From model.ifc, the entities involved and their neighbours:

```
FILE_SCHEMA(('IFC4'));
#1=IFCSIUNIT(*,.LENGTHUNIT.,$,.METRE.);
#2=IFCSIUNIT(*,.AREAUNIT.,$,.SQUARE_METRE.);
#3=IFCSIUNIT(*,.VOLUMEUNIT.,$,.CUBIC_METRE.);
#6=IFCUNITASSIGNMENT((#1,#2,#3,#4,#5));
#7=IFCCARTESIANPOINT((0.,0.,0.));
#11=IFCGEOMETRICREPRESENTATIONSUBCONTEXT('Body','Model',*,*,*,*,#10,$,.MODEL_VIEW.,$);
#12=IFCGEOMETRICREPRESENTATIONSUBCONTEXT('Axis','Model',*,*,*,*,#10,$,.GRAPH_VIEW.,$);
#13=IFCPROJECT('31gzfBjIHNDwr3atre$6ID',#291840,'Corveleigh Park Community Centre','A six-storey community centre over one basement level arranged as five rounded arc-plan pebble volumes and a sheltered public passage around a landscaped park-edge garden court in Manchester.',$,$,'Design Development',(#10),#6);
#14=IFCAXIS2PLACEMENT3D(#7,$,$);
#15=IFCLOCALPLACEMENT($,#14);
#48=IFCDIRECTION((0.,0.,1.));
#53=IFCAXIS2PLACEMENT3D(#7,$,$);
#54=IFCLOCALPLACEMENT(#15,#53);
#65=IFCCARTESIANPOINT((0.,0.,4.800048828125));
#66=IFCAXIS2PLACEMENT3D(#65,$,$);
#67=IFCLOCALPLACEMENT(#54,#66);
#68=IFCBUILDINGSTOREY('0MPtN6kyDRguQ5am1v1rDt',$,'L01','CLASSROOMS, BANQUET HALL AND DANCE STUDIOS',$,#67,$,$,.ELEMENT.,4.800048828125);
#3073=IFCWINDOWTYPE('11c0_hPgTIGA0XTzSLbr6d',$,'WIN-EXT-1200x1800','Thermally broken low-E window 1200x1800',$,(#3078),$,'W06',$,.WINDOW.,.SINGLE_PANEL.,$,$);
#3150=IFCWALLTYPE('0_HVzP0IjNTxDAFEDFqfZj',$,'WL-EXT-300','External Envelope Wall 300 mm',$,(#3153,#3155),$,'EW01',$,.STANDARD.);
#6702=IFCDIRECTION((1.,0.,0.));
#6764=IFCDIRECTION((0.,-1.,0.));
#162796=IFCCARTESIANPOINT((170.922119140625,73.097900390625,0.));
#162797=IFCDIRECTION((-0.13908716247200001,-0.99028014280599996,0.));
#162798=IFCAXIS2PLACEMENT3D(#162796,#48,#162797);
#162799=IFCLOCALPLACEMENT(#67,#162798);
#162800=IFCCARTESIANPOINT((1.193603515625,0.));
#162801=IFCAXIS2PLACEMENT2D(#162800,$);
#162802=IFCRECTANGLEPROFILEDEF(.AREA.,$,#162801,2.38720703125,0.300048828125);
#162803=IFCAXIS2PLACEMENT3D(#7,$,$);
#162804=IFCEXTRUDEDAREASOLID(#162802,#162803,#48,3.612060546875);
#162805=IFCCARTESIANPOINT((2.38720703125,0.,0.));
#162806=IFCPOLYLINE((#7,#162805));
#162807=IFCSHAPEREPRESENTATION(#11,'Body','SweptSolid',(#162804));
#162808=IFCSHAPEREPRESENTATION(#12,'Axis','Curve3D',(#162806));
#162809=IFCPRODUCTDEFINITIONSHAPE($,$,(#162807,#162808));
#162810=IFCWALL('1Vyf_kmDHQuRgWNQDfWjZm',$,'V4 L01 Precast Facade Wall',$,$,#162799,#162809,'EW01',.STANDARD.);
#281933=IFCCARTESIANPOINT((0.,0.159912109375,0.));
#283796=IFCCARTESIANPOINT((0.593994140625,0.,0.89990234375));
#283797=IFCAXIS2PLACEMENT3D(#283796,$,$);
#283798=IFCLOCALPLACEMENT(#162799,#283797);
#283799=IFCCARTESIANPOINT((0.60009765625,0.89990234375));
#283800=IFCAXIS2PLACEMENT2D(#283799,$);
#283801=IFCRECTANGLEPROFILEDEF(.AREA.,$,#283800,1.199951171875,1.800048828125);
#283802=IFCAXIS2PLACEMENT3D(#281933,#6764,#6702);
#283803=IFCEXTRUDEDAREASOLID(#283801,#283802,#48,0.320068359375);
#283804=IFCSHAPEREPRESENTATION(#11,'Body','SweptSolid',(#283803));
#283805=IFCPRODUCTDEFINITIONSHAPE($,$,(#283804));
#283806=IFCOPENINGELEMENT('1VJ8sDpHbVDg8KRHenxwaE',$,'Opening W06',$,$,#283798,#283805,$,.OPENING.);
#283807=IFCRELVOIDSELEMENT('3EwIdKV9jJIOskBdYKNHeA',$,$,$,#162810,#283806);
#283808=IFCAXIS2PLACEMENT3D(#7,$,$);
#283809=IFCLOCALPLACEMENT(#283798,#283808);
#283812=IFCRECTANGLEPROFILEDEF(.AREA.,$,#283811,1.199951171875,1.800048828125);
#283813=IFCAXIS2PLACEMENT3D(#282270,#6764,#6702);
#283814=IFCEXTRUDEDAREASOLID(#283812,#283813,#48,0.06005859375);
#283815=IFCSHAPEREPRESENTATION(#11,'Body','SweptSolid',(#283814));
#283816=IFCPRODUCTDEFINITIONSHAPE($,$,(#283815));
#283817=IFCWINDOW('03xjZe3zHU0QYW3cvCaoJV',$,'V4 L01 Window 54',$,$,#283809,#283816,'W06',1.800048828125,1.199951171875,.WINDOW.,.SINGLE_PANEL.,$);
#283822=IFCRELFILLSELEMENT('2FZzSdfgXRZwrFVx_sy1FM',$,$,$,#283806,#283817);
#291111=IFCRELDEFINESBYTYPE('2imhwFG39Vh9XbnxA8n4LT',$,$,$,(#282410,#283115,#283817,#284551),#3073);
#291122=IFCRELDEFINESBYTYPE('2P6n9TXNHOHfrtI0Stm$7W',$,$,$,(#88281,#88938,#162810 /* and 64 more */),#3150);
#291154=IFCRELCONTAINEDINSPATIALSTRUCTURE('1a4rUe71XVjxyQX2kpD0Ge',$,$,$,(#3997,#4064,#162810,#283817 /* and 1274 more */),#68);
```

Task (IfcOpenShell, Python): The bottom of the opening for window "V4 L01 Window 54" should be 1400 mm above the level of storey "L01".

```python
import numpy as np
import ifcopenshell
import ifcopenshell.api.geometry
import ifcopenshell.geom
import ifcopenshell.util.element
import ifcopenshell.util.placement
import ifcopenshell.util.shape
import ifcopenshell.util.unit

model = ifcopenshell.open("model.ifc")
unit_scale = ifcopenshell.util.unit.calculate_unit_scale(model)

window = model.by_guid("03xjZe3zHU0QYW3cvCaoJV")
opening = window.FillsVoids[0].RelatingOpeningElement
storey = ifcopenshell.util.element.get_container(window, ifc_class="IfcBuildingStorey")
level = ifcopenshell.util.placement.get_local_placement(storey.ObjectPlacement)[2, 3]

# The opening's origin need not be at the sill, so measure its lowest point.
shape = ifcopenshell.geom.create_shape(ifcopenshell.geom.settings(), opening)
bottom = ifcopenshell.util.shape.get_shape_bottom_elevation(shape, shape.geometry) / unit_scale
dz = level + 1.4 / unit_scale - bottom

shift = np.array([0.0, 0.0, dz])
# The window is placed relative to its opening, so it follows when the opening moves.
matrix = ifcopenshell.util.placement.get_local_placement(opening.ObjectPlacement)
matrix[:3, 3] += shift
ifcopenshell.api.geometry.edit_object_placement(
    model, product=opening, matrix=matrix, is_si=False, should_transform_children=True
)

print(f"moved by {dz * unit_scale:+.3f} m")

model.write("model_rev.ifc")
```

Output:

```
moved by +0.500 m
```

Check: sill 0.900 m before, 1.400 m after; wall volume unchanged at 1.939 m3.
